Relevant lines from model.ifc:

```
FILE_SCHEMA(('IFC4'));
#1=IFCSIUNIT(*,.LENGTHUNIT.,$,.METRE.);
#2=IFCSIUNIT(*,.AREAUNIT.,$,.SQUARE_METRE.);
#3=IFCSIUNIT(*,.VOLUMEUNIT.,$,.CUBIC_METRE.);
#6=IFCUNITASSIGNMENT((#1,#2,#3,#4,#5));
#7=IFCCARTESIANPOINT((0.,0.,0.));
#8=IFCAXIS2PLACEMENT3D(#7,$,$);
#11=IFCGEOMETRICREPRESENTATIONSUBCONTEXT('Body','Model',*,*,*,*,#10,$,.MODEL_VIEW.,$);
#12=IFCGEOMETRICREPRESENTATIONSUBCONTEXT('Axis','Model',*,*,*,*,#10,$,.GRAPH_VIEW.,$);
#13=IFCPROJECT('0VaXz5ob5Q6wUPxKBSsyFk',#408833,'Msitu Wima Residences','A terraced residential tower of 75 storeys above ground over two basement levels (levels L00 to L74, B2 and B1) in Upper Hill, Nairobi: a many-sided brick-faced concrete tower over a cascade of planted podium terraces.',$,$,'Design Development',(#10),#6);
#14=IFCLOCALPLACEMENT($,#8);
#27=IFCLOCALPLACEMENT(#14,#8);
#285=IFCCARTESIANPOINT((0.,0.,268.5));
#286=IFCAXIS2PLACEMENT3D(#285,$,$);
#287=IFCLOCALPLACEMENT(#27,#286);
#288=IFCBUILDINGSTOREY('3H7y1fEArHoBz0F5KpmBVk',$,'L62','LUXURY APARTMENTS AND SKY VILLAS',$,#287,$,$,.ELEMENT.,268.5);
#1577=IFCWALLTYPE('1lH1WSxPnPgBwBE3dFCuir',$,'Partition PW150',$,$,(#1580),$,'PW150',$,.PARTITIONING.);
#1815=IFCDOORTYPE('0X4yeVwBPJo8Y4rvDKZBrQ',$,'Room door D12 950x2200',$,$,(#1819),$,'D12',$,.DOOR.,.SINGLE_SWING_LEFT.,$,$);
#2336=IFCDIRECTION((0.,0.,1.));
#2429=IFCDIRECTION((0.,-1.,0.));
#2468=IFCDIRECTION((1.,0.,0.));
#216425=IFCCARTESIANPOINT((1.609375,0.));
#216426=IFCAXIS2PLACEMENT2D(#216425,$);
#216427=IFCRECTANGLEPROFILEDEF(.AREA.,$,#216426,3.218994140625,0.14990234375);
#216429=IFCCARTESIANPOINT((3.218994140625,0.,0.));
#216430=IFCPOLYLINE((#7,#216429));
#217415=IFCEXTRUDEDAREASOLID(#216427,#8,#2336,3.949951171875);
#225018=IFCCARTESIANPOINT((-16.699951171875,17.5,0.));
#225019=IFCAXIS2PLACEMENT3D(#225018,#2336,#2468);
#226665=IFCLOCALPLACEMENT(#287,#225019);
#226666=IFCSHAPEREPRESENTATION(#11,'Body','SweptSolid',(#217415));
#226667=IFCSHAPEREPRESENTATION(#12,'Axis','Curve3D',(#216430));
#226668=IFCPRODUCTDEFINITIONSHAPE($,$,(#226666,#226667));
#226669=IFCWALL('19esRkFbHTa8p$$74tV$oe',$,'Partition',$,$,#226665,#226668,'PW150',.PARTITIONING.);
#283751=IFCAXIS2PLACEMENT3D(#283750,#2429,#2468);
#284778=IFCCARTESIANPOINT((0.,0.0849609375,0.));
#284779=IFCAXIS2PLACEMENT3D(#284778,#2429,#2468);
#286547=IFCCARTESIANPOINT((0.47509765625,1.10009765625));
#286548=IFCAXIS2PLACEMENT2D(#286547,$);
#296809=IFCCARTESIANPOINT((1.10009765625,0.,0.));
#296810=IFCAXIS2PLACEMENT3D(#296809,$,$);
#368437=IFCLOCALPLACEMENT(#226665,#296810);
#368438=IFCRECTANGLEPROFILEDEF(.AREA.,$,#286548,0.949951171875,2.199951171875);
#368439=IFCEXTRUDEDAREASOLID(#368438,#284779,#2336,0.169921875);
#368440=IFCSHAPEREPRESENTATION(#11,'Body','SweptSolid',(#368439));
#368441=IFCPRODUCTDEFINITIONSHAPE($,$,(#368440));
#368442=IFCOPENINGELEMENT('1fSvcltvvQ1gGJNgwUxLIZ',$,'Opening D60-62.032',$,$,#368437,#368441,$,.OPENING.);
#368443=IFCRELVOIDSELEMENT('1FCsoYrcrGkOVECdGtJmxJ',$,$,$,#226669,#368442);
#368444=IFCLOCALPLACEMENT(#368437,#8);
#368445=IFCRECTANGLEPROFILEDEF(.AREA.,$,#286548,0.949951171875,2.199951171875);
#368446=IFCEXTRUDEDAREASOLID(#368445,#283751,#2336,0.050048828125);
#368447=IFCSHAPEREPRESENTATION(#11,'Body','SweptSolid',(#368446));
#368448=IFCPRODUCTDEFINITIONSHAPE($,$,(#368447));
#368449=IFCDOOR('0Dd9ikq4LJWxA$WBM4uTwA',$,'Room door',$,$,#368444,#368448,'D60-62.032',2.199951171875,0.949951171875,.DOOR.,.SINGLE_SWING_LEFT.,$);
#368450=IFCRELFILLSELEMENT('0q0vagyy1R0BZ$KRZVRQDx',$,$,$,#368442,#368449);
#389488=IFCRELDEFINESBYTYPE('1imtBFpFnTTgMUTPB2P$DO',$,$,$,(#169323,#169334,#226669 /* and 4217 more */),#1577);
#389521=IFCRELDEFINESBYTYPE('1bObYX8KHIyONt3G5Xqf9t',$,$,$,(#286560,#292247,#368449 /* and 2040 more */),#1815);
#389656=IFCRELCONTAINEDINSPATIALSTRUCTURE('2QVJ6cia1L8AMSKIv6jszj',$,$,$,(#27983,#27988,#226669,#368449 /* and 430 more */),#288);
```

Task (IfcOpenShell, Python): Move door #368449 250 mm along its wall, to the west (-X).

```python
import ifcopenshell
import ifcopenshell.api.geometry
import ifcopenshell.util.placement

model = ifcopenshell.open("model.ifc")

door = model.by_guid("0Dd9ikq4LJWxA$WBM4uTwA")
opening = door.FillsVoids[0].RelatingOpeningElement
wall = opening.VoidsElements[0].RelatingBuildingElement

wall_matrix = ifcopenshell.util.placement.get_local_placement(wall.ObjectPlacement)
shift = wall_matrix[:3, 0] * -0.25
before = ifcopenshell.util.placement.get_local_placement(door.ObjectPlacement)[:3, 3].copy()

# The door is placed relative to its opening, so it follows when the opening moves.
matrix = ifcopenshell.util.placement.get_local_placement(opening.ObjectPlacement)
matrix[:3, 3] += shift
ifcopenshell.api.geometry.edit_object_placement(
    model, product=opening, matrix=matrix, is_si=False, should_transform_children=True
)

after = ifcopenshell.util.placement.get_local_placement(door.ObjectPlacement)[:3, 3]
print("door moved by", (after - before).round(3) + 0.0)

model.write("model-out.ifc")
```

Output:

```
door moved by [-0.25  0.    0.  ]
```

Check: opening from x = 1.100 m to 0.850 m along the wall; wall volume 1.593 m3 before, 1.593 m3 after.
